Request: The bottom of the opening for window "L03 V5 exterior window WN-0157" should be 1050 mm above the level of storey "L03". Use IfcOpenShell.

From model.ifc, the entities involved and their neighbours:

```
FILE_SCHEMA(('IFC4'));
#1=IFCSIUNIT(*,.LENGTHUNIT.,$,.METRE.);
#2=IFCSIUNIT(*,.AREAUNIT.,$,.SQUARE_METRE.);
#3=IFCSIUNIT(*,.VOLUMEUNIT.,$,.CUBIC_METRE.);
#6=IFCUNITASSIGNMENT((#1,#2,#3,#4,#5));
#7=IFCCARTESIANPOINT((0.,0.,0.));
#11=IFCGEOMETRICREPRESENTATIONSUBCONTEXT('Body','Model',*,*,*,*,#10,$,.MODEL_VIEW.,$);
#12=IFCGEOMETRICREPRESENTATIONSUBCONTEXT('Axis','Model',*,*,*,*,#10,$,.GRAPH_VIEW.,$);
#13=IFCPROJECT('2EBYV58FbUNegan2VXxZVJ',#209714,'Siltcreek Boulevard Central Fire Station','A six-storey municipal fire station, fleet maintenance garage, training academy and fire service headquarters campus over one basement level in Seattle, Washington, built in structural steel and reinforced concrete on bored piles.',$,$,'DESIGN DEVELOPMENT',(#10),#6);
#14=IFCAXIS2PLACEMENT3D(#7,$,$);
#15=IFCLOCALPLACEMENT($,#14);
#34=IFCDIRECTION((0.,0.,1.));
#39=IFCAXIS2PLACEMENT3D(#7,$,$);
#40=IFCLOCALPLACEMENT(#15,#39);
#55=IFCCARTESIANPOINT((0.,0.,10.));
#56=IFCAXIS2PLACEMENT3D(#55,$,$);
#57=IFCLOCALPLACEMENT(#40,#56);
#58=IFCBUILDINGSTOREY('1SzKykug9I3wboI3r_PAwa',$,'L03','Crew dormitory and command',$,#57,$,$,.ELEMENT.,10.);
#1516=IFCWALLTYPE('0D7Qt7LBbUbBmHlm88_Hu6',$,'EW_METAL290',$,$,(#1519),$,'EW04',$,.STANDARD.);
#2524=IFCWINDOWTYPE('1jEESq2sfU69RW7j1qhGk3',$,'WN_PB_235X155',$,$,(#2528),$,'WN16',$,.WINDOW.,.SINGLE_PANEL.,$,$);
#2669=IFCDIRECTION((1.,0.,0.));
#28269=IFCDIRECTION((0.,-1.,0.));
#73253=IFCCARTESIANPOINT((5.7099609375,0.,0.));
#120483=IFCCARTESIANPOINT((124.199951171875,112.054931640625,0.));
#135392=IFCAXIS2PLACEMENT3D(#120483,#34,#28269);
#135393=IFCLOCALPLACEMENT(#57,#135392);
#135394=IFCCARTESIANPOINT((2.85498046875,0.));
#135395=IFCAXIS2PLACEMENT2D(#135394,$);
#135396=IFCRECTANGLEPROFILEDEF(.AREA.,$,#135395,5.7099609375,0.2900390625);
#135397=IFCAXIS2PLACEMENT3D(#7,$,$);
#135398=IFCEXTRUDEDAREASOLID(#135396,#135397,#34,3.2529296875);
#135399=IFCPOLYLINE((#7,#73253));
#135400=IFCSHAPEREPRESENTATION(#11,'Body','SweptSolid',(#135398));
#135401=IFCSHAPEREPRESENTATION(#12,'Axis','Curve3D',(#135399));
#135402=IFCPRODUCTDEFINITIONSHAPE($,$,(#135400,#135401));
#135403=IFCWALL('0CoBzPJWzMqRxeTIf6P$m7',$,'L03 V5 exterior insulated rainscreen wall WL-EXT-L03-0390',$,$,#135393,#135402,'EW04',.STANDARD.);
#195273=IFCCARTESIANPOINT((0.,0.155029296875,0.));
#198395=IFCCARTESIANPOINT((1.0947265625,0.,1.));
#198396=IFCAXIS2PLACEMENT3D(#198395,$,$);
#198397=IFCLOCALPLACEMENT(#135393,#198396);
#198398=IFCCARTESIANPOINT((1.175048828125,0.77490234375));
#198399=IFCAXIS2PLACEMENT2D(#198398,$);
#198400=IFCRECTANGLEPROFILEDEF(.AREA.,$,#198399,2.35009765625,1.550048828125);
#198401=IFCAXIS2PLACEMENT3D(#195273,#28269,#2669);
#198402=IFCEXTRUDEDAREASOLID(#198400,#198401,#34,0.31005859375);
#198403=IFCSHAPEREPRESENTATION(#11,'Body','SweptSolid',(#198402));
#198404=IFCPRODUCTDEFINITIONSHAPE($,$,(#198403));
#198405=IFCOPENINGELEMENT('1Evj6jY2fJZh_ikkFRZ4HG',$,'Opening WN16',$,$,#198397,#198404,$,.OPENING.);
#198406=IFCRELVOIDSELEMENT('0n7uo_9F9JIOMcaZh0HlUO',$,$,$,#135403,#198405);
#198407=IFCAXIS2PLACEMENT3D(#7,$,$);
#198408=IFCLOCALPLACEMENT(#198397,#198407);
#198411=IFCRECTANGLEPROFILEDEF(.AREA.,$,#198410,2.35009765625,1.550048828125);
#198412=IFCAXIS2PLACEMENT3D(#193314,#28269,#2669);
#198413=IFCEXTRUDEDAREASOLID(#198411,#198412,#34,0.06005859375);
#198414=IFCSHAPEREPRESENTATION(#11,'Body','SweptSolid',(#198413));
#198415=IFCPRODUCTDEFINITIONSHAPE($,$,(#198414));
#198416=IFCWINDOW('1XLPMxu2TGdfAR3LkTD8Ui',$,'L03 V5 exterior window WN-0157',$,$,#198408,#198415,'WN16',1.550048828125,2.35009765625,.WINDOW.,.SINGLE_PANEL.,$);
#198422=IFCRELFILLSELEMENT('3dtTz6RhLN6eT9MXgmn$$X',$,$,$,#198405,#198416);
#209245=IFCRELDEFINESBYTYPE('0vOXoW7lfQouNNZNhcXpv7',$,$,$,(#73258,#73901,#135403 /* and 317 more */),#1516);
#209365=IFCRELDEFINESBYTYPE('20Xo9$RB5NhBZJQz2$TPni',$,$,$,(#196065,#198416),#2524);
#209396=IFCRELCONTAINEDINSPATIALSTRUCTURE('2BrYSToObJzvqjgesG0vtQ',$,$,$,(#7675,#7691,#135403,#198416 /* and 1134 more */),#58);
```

```python
import numpy as np
import ifcopenshell
import ifcopenshell.api.geometry
import ifcopenshell.geom
import ifcopenshell.util.element
import ifcopenshell.util.placement
import ifcopenshell.util.shape
import ifcopenshell.util.unit

model = ifcopenshell.open("model.ifc")
unit_scale = ifcopenshell.util.unit.calculate_unit_scale(model)

window = model.by_guid("1XLPMxu2TGdfAR3LkTD8Ui")
opening = window.FillsVoids[0].RelatingOpeningElement
storey = ifcopenshell.util.element.get_container(window, ifc_class="IfcBuildingStorey")
level = ifcopenshell.util.placement.get_local_placement(storey.ObjectPlacement)[2, 3]

# The opening's origin need not be at the sill, so measure its lowest point.
shape = ifcopenshell.geom.create_shape(ifcopenshell.geom.settings(), opening)
bottom = ifcopenshell.util.shape.get_shape_bottom_elevation(shape, shape.geometry) / unit_scale
dz = level + 1.05 / unit_scale - bottom

shift = np.array([0.0, 0.0, dz])
# The window is placed relative to its opening, so it follows when the opening moves.
matrix = ifcopenshell.util.placement.get_local_placement(opening.ObjectPlacement)
matrix[:3, 3] += shift
ifcopenshell.api.geometry.edit_object_placement(
    model, product=opening, matrix=matrix, is_si=False, should_transform_children=True
)

print(f"moved by {dz * unit_scale:+.3f} m")

model.write("model-out.ifc")
```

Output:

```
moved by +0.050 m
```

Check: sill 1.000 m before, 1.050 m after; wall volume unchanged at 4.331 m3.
